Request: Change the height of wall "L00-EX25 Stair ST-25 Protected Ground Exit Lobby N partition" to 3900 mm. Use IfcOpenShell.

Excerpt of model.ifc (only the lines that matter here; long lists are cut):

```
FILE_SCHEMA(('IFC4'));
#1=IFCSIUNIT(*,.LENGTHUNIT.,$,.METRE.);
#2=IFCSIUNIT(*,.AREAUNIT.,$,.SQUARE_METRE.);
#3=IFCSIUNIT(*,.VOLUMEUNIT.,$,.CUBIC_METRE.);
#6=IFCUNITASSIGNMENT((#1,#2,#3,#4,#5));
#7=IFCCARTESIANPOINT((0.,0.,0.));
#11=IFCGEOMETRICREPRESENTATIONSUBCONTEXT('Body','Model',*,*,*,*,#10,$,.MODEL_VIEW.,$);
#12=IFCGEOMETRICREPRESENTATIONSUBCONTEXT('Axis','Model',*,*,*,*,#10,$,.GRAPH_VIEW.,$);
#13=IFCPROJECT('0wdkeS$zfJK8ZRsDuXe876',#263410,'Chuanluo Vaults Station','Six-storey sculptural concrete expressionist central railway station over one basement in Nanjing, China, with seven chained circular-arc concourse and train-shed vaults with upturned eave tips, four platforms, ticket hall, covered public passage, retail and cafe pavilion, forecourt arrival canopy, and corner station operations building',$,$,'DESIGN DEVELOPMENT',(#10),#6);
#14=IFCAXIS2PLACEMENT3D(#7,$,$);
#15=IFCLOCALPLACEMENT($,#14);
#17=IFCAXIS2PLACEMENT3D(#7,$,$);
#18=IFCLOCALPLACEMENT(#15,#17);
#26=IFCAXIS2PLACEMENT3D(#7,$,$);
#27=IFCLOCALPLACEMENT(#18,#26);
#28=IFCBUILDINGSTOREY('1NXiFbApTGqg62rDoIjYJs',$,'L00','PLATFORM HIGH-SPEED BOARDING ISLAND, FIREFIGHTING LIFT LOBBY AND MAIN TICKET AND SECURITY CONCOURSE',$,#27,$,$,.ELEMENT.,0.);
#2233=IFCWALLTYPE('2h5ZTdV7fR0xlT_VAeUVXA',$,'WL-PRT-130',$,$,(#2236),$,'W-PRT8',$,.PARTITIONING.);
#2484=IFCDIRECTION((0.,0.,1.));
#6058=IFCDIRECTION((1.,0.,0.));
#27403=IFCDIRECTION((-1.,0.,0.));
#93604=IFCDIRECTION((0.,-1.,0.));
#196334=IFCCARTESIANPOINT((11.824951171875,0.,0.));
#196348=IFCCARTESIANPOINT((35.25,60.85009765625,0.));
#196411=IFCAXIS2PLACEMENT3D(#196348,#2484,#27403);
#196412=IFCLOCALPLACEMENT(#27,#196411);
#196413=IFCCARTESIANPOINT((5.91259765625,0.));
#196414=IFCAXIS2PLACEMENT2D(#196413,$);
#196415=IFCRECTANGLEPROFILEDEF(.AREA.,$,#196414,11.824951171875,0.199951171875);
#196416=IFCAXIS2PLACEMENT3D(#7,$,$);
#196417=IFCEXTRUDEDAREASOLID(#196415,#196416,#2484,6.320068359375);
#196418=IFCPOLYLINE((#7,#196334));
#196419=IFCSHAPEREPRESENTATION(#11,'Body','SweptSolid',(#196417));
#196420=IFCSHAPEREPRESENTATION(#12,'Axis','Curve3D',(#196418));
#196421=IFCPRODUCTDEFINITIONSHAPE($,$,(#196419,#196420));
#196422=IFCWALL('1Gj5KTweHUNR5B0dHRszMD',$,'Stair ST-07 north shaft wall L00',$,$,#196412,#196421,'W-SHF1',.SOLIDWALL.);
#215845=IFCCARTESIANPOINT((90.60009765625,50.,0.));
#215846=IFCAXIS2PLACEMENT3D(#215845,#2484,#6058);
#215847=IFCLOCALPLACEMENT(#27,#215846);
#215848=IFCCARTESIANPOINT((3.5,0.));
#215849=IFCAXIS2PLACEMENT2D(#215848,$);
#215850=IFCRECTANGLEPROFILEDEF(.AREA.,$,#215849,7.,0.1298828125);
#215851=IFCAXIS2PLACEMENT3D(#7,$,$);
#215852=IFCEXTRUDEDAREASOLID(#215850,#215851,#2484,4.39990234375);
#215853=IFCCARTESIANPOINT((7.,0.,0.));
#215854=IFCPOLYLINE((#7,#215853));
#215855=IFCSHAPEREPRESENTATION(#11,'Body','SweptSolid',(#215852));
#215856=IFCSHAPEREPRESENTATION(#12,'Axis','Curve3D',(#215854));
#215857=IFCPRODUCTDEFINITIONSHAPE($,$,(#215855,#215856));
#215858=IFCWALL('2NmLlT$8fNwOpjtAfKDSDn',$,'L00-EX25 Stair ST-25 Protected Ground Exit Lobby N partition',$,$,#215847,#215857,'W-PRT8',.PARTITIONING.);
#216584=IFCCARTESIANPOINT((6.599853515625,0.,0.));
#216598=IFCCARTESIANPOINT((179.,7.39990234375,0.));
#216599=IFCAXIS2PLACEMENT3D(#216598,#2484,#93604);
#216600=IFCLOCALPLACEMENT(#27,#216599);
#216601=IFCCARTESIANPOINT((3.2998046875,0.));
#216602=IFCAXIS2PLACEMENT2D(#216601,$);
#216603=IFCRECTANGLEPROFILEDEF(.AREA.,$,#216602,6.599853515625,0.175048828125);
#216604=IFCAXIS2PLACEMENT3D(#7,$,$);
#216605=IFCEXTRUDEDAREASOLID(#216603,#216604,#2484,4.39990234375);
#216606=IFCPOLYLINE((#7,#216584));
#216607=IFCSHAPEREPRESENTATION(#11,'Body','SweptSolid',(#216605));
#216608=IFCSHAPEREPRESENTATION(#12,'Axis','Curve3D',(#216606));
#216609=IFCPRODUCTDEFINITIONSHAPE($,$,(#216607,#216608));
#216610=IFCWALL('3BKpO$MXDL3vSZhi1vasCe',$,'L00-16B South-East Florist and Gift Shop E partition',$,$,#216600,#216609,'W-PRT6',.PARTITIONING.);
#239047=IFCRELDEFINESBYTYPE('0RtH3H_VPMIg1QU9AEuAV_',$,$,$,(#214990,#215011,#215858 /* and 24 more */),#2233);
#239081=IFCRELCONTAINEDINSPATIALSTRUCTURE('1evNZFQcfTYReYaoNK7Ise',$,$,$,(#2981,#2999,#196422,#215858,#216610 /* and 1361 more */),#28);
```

```python
import ifcopenshell
import ifcopenshell.geom
import ifcopenshell.util.representation
import ifcopenshell.util.shape
import ifcopenshell.util.unit

model = ifcopenshell.open("model.ifc")
unit_scale = ifcopenshell.util.unit.calculate_unit_scale(model)
settings = ifcopenshell.geom.settings()


def volume(element):
    """Net volume in cubic metres, openings subtracted."""
    shape = ifcopenshell.geom.create_shape(settings, element)
    return ifcopenshell.util.shape.get_volume(shape.geometry)


wall = model.by_id(215858)
before = volume(wall)

body = ifcopenshell.util.representation.get_representation(wall, "Model", "Body")
solid = body.Items[0]
old_height = solid.Depth
solid.Depth = 3.9 / unit_scale
after = volume(wall)

print(f"height {old_height:g} -> {solid.Depth:g}, volume {before:.3f} -> {after:.3f} m3")

model.write("model_rev.ifc")
```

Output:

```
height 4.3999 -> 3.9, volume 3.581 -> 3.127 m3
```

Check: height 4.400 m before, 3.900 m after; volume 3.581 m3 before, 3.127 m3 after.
